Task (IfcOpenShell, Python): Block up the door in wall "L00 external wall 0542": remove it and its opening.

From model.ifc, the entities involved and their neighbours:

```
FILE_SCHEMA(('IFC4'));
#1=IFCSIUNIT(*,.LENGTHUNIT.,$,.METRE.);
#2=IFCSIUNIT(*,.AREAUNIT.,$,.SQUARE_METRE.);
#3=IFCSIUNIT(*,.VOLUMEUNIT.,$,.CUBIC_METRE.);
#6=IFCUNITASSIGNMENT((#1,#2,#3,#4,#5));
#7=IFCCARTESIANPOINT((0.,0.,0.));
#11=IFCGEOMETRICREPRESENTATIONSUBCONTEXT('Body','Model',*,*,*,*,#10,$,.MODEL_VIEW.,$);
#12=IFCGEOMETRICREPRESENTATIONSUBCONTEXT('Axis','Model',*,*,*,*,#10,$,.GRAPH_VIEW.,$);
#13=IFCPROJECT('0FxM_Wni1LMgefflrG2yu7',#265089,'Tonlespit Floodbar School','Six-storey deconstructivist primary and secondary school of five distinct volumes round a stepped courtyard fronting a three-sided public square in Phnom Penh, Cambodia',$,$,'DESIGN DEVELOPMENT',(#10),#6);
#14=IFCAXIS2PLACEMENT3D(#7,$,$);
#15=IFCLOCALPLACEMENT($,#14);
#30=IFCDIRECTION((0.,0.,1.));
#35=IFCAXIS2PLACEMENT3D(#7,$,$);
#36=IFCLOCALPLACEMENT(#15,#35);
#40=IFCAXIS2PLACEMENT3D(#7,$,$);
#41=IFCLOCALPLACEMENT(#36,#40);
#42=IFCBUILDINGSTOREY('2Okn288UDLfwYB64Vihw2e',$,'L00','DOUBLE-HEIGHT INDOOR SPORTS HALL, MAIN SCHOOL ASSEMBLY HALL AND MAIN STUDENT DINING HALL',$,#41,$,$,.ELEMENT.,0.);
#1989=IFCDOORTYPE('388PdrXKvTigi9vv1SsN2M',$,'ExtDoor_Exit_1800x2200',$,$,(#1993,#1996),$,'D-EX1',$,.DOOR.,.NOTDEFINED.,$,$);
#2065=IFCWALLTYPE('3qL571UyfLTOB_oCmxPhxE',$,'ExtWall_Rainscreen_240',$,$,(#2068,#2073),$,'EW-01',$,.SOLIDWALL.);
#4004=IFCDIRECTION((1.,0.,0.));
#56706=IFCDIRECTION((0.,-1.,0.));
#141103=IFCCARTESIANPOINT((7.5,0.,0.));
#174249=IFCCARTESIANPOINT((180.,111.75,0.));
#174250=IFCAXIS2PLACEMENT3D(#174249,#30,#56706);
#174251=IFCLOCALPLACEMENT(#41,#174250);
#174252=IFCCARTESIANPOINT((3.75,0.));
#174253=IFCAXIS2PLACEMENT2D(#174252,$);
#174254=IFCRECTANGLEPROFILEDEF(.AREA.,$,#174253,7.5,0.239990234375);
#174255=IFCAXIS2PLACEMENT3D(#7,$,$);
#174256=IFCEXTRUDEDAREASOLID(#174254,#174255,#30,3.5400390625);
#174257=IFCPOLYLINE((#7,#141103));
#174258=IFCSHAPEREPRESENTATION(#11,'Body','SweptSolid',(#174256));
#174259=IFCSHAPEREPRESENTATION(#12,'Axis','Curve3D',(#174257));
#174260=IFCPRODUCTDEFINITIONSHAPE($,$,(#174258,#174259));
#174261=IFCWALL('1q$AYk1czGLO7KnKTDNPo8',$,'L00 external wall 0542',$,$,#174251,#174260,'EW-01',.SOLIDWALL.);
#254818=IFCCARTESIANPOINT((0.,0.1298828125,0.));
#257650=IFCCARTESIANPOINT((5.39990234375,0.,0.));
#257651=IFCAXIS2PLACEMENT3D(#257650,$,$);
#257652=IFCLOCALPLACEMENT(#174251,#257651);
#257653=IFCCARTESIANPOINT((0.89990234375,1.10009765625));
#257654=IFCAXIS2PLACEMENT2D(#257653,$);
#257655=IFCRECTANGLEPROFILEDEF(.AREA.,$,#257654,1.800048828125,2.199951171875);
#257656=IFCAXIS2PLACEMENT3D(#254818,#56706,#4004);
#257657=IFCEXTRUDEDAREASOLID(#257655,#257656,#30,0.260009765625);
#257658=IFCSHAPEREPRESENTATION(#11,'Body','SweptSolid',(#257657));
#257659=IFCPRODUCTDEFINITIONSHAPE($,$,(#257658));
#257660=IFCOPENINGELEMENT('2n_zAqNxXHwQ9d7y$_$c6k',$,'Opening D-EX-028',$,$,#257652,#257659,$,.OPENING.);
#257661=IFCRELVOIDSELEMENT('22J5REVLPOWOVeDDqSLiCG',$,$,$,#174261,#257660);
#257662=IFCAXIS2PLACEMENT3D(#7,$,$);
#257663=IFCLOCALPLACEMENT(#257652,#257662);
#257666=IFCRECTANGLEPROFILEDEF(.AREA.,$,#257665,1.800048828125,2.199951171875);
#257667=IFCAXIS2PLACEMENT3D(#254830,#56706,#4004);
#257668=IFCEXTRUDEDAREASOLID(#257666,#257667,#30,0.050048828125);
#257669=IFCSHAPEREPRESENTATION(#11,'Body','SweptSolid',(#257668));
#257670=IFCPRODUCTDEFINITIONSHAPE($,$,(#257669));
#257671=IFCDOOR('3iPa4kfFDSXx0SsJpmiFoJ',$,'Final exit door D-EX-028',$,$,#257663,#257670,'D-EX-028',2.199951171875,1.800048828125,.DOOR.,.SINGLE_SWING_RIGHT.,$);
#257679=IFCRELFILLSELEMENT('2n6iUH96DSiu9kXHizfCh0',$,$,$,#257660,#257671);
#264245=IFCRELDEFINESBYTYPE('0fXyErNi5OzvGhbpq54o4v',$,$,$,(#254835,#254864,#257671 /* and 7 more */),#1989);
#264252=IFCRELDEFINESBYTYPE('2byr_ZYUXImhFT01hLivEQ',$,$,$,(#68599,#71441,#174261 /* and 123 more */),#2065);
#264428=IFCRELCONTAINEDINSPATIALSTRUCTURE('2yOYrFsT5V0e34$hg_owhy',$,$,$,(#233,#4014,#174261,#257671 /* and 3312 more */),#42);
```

```python
import ifcopenshell
import ifcopenshell.api.feature
import ifcopenshell.api.root
import ifcopenshell.geom
import ifcopenshell.util.shape

model = ifcopenshell.open("model.ifc")
settings = ifcopenshell.geom.settings()


def volume(element):
    """Net volume in cubic metres, openings subtracted."""
    shape = ifcopenshell.geom.create_shape(settings, element)
    return ifcopenshell.util.shape.get_volume(shape.geometry)


door = model.by_guid("3iPa4kfFDSXx0SsJpmiFoJ")
opening = door.FillsVoids[0].RelatingOpeningElement
wall = opening.VoidsElements[0].RelatingBuildingElement
before = volume(wall)

ifcopenshell.api.root.remove_product(model, product=door)
ifcopenshell.api.feature.remove_feature(model, feature=opening)

after = volume(wall)

print(f"wall volume {before:.3f} -> {after:.3f} m3")

model.write("model-out.ifc")
```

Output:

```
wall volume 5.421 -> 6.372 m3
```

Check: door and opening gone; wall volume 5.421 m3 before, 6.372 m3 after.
